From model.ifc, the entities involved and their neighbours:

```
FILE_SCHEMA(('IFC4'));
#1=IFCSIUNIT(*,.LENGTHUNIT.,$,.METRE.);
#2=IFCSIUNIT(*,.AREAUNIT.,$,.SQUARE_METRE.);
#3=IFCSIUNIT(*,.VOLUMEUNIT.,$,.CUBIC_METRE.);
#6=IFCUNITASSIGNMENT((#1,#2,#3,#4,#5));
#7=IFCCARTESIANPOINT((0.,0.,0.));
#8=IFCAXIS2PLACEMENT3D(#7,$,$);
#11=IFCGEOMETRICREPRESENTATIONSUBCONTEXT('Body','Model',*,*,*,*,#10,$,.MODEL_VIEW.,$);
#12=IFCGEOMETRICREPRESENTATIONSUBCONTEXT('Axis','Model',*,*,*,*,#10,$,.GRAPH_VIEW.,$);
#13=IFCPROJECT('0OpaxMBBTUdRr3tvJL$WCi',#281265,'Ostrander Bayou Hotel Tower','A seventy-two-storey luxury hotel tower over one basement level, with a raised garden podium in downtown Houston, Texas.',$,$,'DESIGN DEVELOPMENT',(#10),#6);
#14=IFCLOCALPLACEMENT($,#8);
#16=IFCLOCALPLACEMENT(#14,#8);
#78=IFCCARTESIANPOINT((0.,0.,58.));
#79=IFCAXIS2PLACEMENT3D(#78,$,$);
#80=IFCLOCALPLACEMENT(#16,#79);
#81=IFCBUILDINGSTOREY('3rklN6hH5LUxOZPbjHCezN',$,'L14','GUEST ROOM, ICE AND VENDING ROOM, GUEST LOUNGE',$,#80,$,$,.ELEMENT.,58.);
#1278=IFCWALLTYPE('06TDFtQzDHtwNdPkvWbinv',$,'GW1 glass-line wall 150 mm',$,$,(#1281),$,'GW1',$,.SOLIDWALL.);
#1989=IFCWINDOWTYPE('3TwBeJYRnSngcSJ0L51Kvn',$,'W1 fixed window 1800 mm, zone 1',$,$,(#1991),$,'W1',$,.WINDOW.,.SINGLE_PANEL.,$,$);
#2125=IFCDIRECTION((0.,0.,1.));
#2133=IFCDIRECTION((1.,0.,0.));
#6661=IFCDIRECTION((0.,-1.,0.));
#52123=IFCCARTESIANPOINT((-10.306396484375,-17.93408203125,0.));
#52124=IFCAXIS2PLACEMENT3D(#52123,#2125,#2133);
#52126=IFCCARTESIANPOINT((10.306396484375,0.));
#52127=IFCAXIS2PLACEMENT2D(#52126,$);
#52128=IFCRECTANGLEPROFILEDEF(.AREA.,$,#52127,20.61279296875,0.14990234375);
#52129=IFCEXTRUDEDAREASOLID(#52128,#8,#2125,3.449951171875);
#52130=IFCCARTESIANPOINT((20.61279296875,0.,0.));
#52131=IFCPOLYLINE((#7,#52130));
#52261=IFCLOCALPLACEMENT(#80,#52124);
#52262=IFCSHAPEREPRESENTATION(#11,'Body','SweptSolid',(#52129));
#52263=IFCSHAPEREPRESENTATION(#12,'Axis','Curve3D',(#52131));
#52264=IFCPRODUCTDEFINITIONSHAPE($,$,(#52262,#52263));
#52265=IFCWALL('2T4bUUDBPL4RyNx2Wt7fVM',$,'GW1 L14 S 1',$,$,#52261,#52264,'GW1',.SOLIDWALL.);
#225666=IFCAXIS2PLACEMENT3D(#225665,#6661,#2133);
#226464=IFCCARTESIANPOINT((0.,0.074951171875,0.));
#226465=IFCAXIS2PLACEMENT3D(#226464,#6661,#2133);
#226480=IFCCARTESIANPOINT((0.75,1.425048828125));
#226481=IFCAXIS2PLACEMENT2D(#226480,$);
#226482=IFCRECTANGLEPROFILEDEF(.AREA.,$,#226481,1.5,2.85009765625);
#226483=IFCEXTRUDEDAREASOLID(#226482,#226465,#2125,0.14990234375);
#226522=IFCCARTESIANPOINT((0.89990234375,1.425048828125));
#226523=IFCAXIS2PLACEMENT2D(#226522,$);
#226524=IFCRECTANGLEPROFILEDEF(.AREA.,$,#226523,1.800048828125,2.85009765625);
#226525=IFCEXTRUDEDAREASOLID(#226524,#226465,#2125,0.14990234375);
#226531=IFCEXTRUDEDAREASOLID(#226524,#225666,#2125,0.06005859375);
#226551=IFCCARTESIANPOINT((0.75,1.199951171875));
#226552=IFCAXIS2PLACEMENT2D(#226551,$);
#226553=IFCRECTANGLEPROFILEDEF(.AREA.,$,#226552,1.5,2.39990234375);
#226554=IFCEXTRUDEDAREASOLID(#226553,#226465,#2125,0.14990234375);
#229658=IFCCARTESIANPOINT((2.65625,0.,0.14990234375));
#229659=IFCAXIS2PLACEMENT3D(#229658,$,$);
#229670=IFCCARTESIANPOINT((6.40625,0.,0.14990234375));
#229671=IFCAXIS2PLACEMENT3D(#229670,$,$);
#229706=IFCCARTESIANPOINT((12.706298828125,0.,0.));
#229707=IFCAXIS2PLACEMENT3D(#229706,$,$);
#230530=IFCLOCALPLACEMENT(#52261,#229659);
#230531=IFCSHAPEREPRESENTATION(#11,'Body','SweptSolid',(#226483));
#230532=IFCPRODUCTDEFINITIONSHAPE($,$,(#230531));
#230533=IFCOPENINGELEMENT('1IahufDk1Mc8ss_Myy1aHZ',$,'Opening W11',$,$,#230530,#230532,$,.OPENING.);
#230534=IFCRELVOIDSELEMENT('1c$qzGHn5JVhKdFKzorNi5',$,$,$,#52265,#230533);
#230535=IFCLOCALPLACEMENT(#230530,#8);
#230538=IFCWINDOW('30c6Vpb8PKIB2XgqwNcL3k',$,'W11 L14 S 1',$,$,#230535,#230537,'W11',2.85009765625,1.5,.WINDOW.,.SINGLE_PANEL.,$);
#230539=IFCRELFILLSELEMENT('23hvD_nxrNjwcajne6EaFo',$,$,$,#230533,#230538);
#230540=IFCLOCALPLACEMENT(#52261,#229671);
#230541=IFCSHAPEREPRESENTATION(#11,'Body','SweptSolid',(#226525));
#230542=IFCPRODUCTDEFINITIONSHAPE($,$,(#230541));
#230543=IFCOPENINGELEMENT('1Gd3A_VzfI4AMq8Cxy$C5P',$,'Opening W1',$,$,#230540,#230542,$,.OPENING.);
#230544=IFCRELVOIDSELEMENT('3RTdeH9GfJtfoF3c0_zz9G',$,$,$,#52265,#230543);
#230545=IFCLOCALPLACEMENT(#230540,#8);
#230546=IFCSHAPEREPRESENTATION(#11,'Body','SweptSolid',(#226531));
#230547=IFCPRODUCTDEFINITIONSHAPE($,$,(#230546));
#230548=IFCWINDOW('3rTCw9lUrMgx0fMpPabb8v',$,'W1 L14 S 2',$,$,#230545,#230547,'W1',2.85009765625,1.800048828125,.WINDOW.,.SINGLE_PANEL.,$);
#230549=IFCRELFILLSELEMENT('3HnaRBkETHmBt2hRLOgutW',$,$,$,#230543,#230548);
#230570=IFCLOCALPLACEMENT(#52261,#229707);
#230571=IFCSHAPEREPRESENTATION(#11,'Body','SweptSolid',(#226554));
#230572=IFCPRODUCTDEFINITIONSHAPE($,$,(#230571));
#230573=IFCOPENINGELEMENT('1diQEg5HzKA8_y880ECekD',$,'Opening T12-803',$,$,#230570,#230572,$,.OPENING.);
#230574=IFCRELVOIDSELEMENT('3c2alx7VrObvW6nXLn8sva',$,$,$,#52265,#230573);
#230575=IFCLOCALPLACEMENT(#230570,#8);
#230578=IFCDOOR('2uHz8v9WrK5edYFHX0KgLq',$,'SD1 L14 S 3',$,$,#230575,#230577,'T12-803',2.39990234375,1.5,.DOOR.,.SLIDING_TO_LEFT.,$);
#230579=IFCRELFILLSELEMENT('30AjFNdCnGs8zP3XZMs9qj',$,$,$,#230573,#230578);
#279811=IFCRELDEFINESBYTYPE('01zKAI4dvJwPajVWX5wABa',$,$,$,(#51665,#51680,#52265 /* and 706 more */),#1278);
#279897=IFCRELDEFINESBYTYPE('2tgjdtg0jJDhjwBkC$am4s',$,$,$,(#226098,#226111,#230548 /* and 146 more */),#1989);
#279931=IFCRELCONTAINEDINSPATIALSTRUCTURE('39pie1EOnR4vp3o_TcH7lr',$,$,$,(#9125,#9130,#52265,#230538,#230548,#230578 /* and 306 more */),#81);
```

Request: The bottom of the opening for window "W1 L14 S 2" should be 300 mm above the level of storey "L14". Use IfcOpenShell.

```python
import numpy as np
import ifcopenshell
import ifcopenshell.api.geometry
import ifcopenshell.geom
import ifcopenshell.util.element
import ifcopenshell.util.placement
import ifcopenshell.util.shape
import ifcopenshell.util.unit

model = ifcopenshell.open("model.ifc")
unit_scale = ifcopenshell.util.unit.calculate_unit_scale(model)

window = model.by_guid("3rTCw9lUrMgx0fMpPabb8v")
opening = window.FillsVoids[0].RelatingOpeningElement
storey = ifcopenshell.util.element.get_container(window, ifc_class="IfcBuildingStorey")
level = ifcopenshell.util.placement.get_local_placement(storey.ObjectPlacement)[2, 3]

# The opening's origin need not be at the sill, so measure its lowest point.
shape = ifcopenshell.geom.create_shape(ifcopenshell.geom.settings(), opening)
bottom = ifcopenshell.util.shape.get_shape_bottom_elevation(shape, shape.geometry) / unit_scale
dz = level + 0.3 - bottom

shift = np.array([0.0, 0.0, dz])
# The window is placed relative to its opening, so it follows when the opening moves.
matrix = ifcopenshell.util.placement.get_local_placement(opening.ObjectPlacement)
matrix[:3, 3] += shift
ifcopenshell.api.geometry.edit_object_placement(
    model, product=opening, matrix=matrix, is_si=False, should_transform_children=True
)

print(f"moved by {dz * unit_scale:+.3f} m")

model.write("model_updated.ifc")
```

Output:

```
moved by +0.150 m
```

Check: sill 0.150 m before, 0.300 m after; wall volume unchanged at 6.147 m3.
